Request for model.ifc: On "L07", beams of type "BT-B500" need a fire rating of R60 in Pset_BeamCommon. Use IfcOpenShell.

First a look at what the model holds.

```python
import ifcopenshell
import ifcopenshell.util.element

model = ifcopenshell.open("model.ifc")
print(model.schema)
storey = next(s for s in model.by_type("IfcBuildingStorey") if s.Name == "L07")
beams = [e for e in ifcopenshell.util.element.get_decomposition(storey) if e.is_a("IfcBeam")]
seen = {}
for e in beams:
    element_type = ifcopenshell.util.element.get_type(e)
    key = (element_type.Name if element_type != e and element_type else None, ifcopenshell.util.element.get_pset(e, "Pset_BeamCommon", "FireRating"))
    seen[key] = seen.get(key, 0) + 1
for (name, value), count in sorted(seen.items(), key=str):
    print(count, "x", name, "|", value)
```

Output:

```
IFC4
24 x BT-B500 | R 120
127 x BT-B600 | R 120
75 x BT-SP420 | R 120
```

```python
import ifcopenshell
import ifcopenshell.api.pset
import ifcopenshell.util.element

model = ifcopenshell.open("model.ifc")

storey = next(s for s in model.by_type("IfcBuildingStorey") if s.Name == "L07")
beams = [e for e in ifcopenshell.util.element.get_decomposition(storey) if e.is_a("IfcBeam")]

count = 0
for e in beams:
    element_type = ifcopenshell.util.element.get_type(e)
    if element_type in (None, e) or element_type.Name != "BT-B500":
        continue
    # add_pset returns the element's existing set when there is one.
    pset = ifcopenshell.api.pset.add_pset(model, product=e, name="Pset_BeamCommon")
    ifcopenshell.api.pset.edit_pset(model, pset=pset, properties={"FireRating": "R60"})
    count += 1

print(count, "beams updated")

model.write("model-out.ifc")
```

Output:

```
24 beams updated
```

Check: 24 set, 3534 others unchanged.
